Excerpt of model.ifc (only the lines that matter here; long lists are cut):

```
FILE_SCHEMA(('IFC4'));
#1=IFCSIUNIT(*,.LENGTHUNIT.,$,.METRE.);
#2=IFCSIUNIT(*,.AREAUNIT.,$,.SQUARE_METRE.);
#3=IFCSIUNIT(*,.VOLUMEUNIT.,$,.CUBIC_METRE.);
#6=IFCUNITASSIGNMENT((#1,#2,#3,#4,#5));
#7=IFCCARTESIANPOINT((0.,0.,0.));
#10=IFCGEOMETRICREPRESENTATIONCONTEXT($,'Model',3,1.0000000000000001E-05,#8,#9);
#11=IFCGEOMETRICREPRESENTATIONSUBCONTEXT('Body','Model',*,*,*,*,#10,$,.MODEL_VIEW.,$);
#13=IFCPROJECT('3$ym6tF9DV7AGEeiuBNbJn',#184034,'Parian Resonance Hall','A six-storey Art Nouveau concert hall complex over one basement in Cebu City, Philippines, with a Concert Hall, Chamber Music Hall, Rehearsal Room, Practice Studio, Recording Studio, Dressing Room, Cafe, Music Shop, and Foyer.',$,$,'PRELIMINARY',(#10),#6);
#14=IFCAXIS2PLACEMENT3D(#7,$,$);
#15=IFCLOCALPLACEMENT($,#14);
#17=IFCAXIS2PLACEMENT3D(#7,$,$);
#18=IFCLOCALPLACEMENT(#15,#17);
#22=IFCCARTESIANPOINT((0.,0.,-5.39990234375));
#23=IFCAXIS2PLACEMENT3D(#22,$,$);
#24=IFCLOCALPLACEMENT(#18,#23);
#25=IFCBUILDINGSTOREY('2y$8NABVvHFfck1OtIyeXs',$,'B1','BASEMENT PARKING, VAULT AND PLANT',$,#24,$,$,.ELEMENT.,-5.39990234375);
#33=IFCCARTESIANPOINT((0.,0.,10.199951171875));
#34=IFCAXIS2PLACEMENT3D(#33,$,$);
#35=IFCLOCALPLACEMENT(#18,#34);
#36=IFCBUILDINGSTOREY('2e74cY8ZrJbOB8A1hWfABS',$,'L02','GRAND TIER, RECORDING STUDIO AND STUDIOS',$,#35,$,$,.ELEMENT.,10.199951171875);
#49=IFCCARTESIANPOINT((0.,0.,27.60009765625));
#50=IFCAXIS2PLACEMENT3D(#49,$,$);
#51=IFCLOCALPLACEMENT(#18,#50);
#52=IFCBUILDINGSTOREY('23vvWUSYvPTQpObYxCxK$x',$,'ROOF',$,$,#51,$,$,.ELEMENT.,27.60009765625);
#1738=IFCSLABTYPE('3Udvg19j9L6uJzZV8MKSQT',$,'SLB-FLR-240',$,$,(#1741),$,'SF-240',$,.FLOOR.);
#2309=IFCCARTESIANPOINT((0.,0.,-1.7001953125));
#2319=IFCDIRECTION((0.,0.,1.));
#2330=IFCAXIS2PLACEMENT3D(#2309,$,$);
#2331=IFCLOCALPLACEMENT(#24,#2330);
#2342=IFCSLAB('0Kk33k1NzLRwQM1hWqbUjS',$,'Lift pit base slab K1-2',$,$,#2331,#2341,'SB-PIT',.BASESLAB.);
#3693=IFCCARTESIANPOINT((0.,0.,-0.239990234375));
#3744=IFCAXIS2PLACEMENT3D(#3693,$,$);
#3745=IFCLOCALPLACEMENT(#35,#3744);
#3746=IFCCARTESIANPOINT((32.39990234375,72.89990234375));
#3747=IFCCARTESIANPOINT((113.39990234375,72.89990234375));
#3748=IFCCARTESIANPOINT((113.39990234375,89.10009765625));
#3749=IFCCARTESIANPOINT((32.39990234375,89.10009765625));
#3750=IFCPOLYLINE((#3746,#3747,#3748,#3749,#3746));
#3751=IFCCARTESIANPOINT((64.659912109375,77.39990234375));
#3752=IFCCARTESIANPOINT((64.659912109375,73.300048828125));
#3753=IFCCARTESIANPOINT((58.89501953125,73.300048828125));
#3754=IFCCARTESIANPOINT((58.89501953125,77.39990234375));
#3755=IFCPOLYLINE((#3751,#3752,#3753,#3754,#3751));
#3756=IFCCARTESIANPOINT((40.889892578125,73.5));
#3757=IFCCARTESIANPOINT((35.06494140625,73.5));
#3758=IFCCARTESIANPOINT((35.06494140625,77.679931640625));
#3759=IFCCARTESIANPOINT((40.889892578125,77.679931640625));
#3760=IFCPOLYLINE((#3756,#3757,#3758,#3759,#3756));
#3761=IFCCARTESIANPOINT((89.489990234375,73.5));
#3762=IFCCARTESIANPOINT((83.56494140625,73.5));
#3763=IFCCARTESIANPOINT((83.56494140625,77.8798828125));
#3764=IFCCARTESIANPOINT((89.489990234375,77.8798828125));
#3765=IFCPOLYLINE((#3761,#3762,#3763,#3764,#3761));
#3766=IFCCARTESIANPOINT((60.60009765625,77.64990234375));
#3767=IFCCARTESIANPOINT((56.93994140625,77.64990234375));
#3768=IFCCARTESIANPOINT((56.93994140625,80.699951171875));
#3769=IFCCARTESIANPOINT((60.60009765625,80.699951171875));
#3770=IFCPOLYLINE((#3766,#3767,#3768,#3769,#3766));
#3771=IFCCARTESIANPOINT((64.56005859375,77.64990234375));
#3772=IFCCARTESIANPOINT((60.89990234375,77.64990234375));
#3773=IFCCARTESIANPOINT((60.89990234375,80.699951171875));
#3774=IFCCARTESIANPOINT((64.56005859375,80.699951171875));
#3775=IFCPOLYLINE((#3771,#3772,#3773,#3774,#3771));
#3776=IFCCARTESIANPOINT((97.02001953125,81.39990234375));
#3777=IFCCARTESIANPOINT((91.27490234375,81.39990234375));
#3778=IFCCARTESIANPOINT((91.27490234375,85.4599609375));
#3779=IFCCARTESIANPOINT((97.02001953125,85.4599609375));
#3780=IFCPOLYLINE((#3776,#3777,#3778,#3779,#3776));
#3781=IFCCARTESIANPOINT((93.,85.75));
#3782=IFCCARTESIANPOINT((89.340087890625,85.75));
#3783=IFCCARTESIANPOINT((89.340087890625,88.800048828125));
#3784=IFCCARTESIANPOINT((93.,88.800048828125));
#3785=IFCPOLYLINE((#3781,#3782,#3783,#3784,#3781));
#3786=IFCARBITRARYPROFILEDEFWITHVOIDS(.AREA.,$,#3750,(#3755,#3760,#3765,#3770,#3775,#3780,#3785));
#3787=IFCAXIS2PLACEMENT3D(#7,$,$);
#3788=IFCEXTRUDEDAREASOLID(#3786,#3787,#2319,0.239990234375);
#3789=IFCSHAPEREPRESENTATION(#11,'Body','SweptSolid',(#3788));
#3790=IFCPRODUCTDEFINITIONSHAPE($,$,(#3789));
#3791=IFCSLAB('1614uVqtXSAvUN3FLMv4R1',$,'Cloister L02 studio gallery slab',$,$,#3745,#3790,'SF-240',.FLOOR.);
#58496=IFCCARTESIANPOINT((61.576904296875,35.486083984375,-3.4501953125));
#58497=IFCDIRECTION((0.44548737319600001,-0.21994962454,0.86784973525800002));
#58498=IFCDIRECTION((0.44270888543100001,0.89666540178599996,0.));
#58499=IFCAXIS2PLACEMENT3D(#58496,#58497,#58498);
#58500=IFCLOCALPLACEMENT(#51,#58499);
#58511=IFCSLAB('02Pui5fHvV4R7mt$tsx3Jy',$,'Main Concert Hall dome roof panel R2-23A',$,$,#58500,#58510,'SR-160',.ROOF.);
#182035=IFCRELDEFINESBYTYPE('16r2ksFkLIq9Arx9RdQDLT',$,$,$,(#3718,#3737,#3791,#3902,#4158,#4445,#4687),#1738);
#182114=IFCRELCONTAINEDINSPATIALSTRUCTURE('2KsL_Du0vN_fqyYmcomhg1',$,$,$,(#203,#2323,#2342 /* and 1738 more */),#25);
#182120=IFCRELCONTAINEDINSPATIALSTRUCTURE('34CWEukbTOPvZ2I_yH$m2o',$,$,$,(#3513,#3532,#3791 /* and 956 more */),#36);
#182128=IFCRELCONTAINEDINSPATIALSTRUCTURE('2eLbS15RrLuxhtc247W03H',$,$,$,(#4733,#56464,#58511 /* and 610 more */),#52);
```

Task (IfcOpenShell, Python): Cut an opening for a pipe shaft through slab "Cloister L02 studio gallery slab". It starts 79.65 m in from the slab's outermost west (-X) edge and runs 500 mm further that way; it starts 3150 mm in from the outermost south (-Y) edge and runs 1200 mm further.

```python
import numpy as np
import ifcopenshell
import ifcopenshell.api.feature
import ifcopenshell.api.geometry
import ifcopenshell.api.root
import ifcopenshell.geom
import ifcopenshell.util.placement
import ifcopenshell.util.representation
import ifcopenshell.util.shape
import ifcopenshell.util.unit

model = ifcopenshell.open("model.ifc")
unit_scale = ifcopenshell.util.unit.calculate_unit_scale(model)
settings = ifcopenshell.geom.settings()


def volume(element):
    """Net volume in cubic metres, openings subtracted."""
    shape = ifcopenshell.geom.create_shape(settings, element)
    return ifcopenshell.util.shape.get_volume(shape.geometry)


slab = model.by_guid("1614uVqtXSAvUN3FLMv4R1")
before = volume(slab)

# Extent in the slab's own axes, in metres. The edges named are its -X and -Y sides.
slab_shape = ifcopenshell.geom.create_shape(settings, slab)
vertices = ifcopenshell.util.shape.get_vertices(slab_shape.geometry)
x_min, y_min, bottom = vertices.min(axis=0)
top = vertices[:, 2].max()

opening = ifcopenshell.api.root.create_entity(model, ifc_class="IfcOpeningElement", name="Pipe shaft opening", predefined_type="OPENING")
context = ifcopenshell.util.representation.get_context(model, "Model", "Body", "MODEL_VIEW")
width, depth = 0.5, 1.2
outline = [(0.0, 0.0), (width, 0.0), (width, depth), (0.0, depth), (0.0, 0.0)]
# Overshoot both faces by 50 mm so the cut is clean.
shape = ifcopenshell.api.geometry.add_slab_representation(
    model, context=context, depth=top - bottom + 0.1, polyline=outline
)
ifcopenshell.api.geometry.assign_representation(model, product=opening, representation=shape)

matrix = ifcopenshell.util.placement.get_local_placement(slab.ObjectPlacement)
matrix[:, 3] = matrix @ np.append(np.array([x_min + 79.65, y_min + 3.15, bottom - 0.05]) / unit_scale, 1.0)
ifcopenshell.api.geometry.edit_object_placement(model, product=opening, matrix=matrix, is_si=False)
ifcopenshell.api.feature.add_feature(model, feature=opening, element=slab)

after = volume(slab)

print(f"slab volume {before:.3f} -> {after:.3f} m3")

model.write("model_updated.ifc")
```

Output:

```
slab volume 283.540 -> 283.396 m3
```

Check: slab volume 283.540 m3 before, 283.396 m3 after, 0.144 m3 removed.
